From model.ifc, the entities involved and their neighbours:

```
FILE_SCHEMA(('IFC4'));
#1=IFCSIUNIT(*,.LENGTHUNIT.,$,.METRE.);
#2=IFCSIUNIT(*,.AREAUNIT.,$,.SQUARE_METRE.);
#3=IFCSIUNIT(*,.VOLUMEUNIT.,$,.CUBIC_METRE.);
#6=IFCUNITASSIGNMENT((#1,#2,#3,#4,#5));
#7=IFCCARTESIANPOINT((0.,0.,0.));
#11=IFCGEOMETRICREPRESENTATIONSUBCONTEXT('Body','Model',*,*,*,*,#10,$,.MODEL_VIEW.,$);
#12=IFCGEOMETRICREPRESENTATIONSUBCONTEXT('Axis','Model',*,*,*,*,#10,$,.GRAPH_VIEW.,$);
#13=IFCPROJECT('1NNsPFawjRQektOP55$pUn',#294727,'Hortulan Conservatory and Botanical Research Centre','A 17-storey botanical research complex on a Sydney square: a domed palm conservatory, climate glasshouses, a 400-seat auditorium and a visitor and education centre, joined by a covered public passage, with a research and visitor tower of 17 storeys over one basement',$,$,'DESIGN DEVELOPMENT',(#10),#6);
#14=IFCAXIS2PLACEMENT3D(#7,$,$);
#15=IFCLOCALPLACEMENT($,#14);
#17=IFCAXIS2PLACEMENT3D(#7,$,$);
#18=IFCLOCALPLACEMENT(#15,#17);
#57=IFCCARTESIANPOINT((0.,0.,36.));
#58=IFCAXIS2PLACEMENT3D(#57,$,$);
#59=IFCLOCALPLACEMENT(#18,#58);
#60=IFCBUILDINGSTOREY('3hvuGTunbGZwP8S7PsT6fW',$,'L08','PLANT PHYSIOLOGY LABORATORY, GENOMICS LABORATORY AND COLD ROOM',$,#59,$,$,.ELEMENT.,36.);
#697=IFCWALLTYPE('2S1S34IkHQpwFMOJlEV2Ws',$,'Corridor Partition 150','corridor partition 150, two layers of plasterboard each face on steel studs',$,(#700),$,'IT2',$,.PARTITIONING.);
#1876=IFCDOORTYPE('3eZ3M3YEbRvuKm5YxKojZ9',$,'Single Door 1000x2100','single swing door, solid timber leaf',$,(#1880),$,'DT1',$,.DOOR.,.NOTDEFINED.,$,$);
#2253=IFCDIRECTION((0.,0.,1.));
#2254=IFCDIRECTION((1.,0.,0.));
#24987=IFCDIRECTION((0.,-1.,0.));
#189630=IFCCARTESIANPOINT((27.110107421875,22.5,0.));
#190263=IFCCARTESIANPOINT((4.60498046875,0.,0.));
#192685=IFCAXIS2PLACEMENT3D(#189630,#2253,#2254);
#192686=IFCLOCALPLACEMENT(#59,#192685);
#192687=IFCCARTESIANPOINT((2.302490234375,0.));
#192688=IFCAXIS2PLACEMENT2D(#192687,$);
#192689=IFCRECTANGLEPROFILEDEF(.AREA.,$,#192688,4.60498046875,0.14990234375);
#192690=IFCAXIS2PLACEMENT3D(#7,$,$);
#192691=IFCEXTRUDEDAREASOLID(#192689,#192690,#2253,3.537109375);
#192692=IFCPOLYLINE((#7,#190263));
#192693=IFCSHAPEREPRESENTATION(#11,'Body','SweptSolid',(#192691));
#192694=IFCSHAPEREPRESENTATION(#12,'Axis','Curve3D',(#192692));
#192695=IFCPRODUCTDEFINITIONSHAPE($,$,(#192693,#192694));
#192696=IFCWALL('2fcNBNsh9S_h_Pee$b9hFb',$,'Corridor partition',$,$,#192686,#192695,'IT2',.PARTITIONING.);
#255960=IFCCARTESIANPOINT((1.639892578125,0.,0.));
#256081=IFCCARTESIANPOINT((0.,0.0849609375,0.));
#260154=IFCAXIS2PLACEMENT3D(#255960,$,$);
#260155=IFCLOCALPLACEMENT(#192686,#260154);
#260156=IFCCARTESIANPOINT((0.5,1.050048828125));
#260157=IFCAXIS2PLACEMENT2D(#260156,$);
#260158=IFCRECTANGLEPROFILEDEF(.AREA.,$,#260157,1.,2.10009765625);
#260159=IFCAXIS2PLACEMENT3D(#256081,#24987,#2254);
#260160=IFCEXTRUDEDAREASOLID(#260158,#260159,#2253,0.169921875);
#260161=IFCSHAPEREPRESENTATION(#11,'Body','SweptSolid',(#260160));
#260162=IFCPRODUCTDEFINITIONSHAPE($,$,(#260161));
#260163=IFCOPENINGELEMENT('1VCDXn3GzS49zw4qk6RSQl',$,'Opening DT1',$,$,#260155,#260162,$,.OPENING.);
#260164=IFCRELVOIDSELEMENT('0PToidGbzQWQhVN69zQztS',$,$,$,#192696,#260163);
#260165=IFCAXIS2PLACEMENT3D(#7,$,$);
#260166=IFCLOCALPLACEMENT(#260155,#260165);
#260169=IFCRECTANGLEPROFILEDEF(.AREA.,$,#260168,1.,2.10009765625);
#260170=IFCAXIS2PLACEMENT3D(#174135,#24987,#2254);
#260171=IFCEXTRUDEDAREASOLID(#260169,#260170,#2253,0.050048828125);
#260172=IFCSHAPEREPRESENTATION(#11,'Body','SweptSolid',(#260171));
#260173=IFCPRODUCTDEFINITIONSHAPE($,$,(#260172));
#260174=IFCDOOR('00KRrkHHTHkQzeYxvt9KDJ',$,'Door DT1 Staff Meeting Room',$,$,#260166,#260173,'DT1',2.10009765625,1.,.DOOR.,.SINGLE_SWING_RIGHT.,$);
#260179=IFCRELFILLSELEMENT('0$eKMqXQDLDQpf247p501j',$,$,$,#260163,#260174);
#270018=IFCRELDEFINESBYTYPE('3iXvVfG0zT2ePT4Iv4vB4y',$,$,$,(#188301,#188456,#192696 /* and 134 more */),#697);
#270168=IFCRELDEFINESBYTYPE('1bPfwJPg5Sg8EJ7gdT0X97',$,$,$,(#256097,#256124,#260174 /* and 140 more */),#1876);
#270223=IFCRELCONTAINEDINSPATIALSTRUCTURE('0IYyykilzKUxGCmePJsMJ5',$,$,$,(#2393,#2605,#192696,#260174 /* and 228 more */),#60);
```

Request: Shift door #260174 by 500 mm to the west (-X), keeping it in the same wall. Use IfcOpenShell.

```python
import ifcopenshell
import ifcopenshell.api.geometry
import ifcopenshell.util.placement
import ifcopenshell.util.unit

model = ifcopenshell.open("model.ifc")
unit_scale = ifcopenshell.util.unit.calculate_unit_scale(model)

door = model.by_guid("00KRrkHHTHkQzeYxvt9KDJ")
opening = door.FillsVoids[0].RelatingOpeningElement
wall = opening.VoidsElements[0].RelatingBuildingElement

wall_matrix = ifcopenshell.util.placement.get_local_placement(wall.ObjectPlacement)
shift = wall_matrix[:3, 0] * -0.5 / unit_scale
before = ifcopenshell.util.placement.get_local_placement(door.ObjectPlacement)[:3, 3].copy()

# The door is placed relative to its opening, so it follows when the opening moves.
matrix = ifcopenshell.util.placement.get_local_placement(opening.ObjectPlacement)
matrix[:3, 3] += shift
ifcopenshell.api.geometry.edit_object_placement(
    model, product=opening, matrix=matrix, is_si=False, should_transform_children=True
)

after = ifcopenshell.util.placement.get_local_placement(door.ObjectPlacement)[:3, 3]
print("door moved by", (after - before).round(3) + 0.0)

model.write("model_rev.ifc")
```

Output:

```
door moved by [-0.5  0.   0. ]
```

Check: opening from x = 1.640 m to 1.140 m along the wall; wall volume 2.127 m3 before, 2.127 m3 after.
